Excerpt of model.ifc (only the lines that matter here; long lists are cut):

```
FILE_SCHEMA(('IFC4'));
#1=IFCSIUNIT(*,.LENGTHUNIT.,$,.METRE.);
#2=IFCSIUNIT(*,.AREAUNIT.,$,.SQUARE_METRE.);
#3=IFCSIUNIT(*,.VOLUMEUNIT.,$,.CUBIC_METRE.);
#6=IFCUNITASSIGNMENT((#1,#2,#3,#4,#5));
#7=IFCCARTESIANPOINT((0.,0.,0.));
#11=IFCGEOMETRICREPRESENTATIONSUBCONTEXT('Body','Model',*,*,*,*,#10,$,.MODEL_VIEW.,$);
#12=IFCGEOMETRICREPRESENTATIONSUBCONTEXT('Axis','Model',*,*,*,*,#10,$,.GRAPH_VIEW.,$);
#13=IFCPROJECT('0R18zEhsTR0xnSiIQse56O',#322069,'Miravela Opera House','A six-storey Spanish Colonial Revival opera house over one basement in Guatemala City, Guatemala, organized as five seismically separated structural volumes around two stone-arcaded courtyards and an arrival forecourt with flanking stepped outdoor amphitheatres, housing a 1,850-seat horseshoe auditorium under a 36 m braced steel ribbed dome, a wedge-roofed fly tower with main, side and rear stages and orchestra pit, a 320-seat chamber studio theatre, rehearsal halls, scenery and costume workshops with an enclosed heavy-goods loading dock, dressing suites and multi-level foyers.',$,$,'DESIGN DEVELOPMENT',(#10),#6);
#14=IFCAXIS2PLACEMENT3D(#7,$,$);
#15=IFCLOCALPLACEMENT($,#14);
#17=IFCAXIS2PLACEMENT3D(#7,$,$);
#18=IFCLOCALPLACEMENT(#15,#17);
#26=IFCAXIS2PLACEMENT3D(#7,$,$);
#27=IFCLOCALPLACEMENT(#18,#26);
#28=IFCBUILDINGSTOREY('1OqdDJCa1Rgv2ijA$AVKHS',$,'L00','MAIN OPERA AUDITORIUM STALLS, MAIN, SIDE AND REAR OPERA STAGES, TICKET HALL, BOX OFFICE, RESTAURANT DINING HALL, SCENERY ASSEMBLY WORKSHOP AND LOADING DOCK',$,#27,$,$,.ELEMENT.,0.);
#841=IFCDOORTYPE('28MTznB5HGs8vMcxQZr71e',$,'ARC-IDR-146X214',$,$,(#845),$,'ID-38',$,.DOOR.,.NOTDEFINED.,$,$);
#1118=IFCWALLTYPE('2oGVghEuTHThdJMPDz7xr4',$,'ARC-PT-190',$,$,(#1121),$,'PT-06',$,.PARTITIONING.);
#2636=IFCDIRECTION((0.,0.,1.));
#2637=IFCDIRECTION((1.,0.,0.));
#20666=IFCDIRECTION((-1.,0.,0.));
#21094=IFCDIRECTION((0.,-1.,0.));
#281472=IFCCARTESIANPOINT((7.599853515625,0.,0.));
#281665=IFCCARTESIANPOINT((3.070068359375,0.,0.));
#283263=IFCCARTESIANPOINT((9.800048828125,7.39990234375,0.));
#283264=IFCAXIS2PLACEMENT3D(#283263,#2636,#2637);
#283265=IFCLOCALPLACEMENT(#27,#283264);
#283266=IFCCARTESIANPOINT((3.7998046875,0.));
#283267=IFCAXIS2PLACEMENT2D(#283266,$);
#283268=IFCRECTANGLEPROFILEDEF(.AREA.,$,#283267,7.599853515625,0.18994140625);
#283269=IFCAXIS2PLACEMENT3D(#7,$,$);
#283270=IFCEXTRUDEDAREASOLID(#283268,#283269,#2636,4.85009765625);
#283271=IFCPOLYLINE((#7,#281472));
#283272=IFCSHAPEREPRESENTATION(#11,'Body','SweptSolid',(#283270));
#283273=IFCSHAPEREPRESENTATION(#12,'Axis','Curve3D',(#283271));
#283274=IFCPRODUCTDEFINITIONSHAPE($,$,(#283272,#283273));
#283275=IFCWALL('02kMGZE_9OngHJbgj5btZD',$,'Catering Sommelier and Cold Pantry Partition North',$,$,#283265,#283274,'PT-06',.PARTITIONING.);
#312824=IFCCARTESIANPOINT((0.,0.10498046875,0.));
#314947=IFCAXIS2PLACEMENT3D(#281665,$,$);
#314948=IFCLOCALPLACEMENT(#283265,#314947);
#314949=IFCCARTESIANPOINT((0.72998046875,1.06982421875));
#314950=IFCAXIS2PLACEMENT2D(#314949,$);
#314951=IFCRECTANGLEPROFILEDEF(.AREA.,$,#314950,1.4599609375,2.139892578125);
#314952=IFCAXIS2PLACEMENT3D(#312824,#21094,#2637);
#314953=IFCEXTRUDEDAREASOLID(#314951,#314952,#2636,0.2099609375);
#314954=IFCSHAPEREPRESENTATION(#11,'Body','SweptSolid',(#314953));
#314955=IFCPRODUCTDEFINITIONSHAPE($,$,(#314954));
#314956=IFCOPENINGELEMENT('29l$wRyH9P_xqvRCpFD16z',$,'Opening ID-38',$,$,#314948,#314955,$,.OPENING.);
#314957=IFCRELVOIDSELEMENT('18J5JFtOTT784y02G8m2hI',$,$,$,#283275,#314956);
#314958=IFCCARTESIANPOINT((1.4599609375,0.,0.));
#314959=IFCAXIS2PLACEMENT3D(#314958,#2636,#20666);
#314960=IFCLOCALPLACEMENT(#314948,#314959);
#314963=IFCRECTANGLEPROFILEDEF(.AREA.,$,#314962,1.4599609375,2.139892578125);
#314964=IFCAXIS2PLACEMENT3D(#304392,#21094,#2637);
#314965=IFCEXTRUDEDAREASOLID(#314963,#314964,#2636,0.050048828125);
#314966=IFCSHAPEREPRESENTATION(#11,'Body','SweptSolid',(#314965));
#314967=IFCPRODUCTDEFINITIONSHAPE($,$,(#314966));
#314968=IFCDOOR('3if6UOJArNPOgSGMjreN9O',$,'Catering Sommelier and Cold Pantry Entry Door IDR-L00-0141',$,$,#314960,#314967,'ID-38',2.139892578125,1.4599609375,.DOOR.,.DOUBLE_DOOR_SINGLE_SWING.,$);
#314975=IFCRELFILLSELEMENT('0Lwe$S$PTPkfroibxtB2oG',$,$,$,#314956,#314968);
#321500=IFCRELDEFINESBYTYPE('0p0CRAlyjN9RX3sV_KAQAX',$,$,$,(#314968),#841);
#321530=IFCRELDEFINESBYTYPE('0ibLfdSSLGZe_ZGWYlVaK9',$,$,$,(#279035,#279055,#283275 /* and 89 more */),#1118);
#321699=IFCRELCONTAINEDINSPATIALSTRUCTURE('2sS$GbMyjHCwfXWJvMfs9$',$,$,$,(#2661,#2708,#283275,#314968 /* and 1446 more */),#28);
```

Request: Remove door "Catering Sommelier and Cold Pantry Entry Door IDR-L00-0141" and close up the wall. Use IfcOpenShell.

```python
import ifcopenshell
import ifcopenshell.api.feature
import ifcopenshell.api.root
import ifcopenshell.geom
import ifcopenshell.util.shape

model = ifcopenshell.open("model.ifc")
settings = ifcopenshell.geom.settings()


def volume(element):
    """Net volume in cubic metres, openings subtracted."""
    shape = ifcopenshell.geom.create_shape(settings, element)
    return ifcopenshell.util.shape.get_volume(shape.geometry)


door = model.by_guid("3if6UOJArNPOgSGMjreN9O")
opening = door.FillsVoids[0].RelatingOpeningElement
wall = opening.VoidsElements[0].RelatingBuildingElement
before = volume(wall)

ifcopenshell.api.root.remove_product(model, product=door)
ifcopenshell.api.feature.remove_feature(model, feature=opening)

after = volume(wall)

print(f"wall volume {before:.3f} -> {after:.3f} m3")

model.write("model_updated.ifc")
```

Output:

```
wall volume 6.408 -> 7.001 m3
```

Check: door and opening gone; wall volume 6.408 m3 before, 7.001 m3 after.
